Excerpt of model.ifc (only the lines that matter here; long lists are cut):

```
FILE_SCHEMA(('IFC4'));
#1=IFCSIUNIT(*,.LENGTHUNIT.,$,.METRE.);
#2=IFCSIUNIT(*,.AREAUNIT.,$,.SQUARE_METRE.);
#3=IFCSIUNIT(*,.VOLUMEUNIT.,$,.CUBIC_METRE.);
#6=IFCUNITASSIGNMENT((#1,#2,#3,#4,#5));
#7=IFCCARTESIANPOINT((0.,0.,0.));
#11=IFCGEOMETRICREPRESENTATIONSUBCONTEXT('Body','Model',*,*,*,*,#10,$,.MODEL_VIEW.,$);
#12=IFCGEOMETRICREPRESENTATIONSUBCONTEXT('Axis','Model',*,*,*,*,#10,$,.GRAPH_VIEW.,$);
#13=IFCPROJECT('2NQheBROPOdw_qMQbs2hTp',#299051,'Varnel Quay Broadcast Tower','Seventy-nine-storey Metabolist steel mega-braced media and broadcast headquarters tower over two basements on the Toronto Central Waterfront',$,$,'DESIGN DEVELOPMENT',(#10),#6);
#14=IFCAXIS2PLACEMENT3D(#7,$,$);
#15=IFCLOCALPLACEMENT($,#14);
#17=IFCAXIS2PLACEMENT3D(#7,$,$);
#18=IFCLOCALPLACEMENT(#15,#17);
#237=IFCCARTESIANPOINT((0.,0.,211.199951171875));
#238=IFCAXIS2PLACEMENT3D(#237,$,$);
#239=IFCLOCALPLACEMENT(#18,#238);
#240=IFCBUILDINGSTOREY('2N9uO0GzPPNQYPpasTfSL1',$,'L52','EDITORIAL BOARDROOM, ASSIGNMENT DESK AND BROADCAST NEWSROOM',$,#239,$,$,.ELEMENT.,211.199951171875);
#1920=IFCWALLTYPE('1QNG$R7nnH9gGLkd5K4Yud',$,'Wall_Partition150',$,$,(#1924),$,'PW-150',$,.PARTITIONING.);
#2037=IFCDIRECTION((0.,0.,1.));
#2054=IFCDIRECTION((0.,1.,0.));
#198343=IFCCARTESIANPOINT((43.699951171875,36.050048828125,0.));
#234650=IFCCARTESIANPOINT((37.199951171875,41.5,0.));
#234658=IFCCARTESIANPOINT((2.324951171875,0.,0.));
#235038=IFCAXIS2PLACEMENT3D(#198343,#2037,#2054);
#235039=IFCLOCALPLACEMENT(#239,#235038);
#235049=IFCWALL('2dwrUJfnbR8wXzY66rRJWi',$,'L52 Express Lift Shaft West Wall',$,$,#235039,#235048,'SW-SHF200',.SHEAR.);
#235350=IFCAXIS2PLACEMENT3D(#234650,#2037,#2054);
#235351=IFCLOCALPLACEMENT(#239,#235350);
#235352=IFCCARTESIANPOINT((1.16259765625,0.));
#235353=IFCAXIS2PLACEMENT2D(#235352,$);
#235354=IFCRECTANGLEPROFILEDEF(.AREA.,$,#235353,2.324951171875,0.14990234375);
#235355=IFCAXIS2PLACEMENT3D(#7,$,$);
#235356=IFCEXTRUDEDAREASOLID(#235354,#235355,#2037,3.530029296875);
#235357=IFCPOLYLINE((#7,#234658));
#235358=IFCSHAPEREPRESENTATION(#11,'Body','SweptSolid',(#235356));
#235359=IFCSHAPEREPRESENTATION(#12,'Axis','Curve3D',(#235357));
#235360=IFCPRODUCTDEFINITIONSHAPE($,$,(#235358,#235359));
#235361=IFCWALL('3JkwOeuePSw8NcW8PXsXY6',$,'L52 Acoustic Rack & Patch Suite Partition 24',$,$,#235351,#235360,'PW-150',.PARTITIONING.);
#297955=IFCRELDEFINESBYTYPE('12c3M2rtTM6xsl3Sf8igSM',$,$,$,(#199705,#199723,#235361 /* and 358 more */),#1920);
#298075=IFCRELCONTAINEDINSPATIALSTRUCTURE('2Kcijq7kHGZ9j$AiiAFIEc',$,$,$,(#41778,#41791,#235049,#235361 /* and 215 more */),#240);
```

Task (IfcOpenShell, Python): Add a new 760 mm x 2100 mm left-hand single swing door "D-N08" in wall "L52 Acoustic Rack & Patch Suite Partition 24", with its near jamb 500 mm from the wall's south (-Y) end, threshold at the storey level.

```python
import numpy as np
import ifcopenshell
import ifcopenshell.api.feature
import ifcopenshell.api.geometry
import ifcopenshell.api.root
import ifcopenshell.api.spatial
import ifcopenshell.geom
import ifcopenshell.util.element
import ifcopenshell.util.placement
import ifcopenshell.util.representation
import ifcopenshell.util.shape
import ifcopenshell.util.unit

model = ifcopenshell.open("model.ifc")
unit_scale = ifcopenshell.util.unit.calculate_unit_scale(model)
settings = ifcopenshell.geom.settings()


def volume(element):
    """Net volume in cubic metres, openings subtracted."""
    shape = ifcopenshell.geom.create_shape(settings, element)
    return ifcopenshell.util.shape.get_volume(shape.geometry)


wall = model.by_id(235361)
storey = ifcopenshell.util.element.get_container(wall, ifc_class="IfcBuildingStorey")
context = ifcopenshell.util.representation.get_context(model, "Model", "Body", "MODEL_VIEW")
before = volume(wall)

width, height, from_end, sill = 0.76, 2.1, 0.5, 0.0  # metres

# The wall runs along its own X axis, and the end named is its -X end.
wall_shape = ifcopenshell.geom.create_shape(settings, wall)
x, y, z = ifcopenshell.util.shape.get_vertices(wall_shape.geometry).T
start = x.min() + from_end
face, thickness = float(y.min()), float(y.max() - y.min())
wall_matrix = ifcopenshell.util.placement.get_local_placement(wall.ObjectPlacement)
level = ifcopenshell.util.placement.get_local_placement(storey.ObjectPlacement)[2, 3]


def in_wall(x, y):
    """Placement at x, y metres in the wall's axes, at sill height."""
    matrix = wall_matrix.copy()
    matrix[:, 3] = wall_matrix @ np.array([x / unit_scale, y / unit_scale, 0.0, 1.0])
    matrix[2, 3] = level + sill / unit_scale
    return matrix


# Opening: a box that overshoots both wall faces by 50 mm.
opening = ifcopenshell.api.root.create_entity(model, ifc_class="IfcOpeningElement", predefined_type="OPENING")
box = ifcopenshell.api.geometry.add_wall_representation(
    model, context=context, length=width, height=height, thickness=thickness + 0.1
)
ifcopenshell.api.geometry.assign_representation(model, product=opening, representation=box)
ifcopenshell.api.geometry.edit_object_placement(model, product=opening, matrix=in_wall(start, face - 0.05), is_si=False)
ifcopenshell.api.feature.add_feature(model, feature=opening, element=wall)

door = ifcopenshell.api.root.create_entity(model, ifc_class="IfcDoor", name="D-N08", predefined_type="DOOR")
door.OverallWidth, door.OverallHeight = width / unit_scale, height / unit_scale
door.OperationType = "SINGLE_SWING_LEFT"
body = ifcopenshell.api.geometry.add_door_representation(
    model,
    context=context,
    overall_width=door.OverallWidth,
    overall_height=door.OverallHeight,
    operation_type="SINGLE_SWING_LEFT",
    lining_properties={"LiningDepth": thickness / unit_scale, "ThresholdDepth": thickness / unit_scale},
)
ifcopenshell.api.geometry.assign_representation(model, product=door, representation=body)
ifcopenshell.api.spatial.assign_container(model, products=[door], relating_structure=storey)
ifcopenshell.api.feature.add_filling(model, opening=opening, element=door)

# The lining spans the wall, so the door starts at the wall face.
ifcopenshell.api.geometry.edit_object_placement(model, product=door, matrix=in_wall(start, face), is_si=False)

after = volume(wall)

print(f"wall volume {before:.3f} -> {after:.3f} m3")

model.write("model_edited.ifc")
```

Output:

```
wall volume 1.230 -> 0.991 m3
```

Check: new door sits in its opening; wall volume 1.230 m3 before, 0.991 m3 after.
